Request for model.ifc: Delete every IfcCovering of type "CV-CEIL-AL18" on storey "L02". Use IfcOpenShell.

First a look at what the model holds.

```python
import ifcopenshell
import ifcopenshell.util.element

model = ifcopenshell.open("model.ifc")
print(model.schema)
storey = next(s for s in model.by_type("IfcBuildingStorey") if s.Name == "L02")
coverings = [e for e in ifcopenshell.util.element.get_decomposition(storey) if e.is_a("IfcCovering")]
seen = {}
for e in coverings:
    element_type = ifcopenshell.util.element.get_type(e)
    name = element_type.Name if element_type not in (None, e) else None
    seen[name] = seen.get(name, 0) + 1
for name, count in sorted(seen.items(), key=str):
    print(count, "x", name)
```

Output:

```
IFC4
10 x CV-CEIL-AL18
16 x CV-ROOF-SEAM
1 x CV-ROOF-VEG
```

```python
import ifcopenshell
import ifcopenshell.api.root
import ifcopenshell.util.element

model = ifcopenshell.open("model.ifc")

storey = next(s for s in model.by_type("IfcBuildingStorey") if s.Name == "L02")
coverings = [e for e in ifcopenshell.util.element.get_decomposition(storey) if e.is_a("IfcCovering")]
targets = [e for e in coverings if (t := ifcopenshell.util.element.get_type(e)) not in (None, e) and t.Name == "CV-CEIL-AL18"]

for e in targets:
    ifcopenshell.api.root.remove_product(model, product=e)
print(len(targets), "removed")

model.write("model_updated.ifc")
```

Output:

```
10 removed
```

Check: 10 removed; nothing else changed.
